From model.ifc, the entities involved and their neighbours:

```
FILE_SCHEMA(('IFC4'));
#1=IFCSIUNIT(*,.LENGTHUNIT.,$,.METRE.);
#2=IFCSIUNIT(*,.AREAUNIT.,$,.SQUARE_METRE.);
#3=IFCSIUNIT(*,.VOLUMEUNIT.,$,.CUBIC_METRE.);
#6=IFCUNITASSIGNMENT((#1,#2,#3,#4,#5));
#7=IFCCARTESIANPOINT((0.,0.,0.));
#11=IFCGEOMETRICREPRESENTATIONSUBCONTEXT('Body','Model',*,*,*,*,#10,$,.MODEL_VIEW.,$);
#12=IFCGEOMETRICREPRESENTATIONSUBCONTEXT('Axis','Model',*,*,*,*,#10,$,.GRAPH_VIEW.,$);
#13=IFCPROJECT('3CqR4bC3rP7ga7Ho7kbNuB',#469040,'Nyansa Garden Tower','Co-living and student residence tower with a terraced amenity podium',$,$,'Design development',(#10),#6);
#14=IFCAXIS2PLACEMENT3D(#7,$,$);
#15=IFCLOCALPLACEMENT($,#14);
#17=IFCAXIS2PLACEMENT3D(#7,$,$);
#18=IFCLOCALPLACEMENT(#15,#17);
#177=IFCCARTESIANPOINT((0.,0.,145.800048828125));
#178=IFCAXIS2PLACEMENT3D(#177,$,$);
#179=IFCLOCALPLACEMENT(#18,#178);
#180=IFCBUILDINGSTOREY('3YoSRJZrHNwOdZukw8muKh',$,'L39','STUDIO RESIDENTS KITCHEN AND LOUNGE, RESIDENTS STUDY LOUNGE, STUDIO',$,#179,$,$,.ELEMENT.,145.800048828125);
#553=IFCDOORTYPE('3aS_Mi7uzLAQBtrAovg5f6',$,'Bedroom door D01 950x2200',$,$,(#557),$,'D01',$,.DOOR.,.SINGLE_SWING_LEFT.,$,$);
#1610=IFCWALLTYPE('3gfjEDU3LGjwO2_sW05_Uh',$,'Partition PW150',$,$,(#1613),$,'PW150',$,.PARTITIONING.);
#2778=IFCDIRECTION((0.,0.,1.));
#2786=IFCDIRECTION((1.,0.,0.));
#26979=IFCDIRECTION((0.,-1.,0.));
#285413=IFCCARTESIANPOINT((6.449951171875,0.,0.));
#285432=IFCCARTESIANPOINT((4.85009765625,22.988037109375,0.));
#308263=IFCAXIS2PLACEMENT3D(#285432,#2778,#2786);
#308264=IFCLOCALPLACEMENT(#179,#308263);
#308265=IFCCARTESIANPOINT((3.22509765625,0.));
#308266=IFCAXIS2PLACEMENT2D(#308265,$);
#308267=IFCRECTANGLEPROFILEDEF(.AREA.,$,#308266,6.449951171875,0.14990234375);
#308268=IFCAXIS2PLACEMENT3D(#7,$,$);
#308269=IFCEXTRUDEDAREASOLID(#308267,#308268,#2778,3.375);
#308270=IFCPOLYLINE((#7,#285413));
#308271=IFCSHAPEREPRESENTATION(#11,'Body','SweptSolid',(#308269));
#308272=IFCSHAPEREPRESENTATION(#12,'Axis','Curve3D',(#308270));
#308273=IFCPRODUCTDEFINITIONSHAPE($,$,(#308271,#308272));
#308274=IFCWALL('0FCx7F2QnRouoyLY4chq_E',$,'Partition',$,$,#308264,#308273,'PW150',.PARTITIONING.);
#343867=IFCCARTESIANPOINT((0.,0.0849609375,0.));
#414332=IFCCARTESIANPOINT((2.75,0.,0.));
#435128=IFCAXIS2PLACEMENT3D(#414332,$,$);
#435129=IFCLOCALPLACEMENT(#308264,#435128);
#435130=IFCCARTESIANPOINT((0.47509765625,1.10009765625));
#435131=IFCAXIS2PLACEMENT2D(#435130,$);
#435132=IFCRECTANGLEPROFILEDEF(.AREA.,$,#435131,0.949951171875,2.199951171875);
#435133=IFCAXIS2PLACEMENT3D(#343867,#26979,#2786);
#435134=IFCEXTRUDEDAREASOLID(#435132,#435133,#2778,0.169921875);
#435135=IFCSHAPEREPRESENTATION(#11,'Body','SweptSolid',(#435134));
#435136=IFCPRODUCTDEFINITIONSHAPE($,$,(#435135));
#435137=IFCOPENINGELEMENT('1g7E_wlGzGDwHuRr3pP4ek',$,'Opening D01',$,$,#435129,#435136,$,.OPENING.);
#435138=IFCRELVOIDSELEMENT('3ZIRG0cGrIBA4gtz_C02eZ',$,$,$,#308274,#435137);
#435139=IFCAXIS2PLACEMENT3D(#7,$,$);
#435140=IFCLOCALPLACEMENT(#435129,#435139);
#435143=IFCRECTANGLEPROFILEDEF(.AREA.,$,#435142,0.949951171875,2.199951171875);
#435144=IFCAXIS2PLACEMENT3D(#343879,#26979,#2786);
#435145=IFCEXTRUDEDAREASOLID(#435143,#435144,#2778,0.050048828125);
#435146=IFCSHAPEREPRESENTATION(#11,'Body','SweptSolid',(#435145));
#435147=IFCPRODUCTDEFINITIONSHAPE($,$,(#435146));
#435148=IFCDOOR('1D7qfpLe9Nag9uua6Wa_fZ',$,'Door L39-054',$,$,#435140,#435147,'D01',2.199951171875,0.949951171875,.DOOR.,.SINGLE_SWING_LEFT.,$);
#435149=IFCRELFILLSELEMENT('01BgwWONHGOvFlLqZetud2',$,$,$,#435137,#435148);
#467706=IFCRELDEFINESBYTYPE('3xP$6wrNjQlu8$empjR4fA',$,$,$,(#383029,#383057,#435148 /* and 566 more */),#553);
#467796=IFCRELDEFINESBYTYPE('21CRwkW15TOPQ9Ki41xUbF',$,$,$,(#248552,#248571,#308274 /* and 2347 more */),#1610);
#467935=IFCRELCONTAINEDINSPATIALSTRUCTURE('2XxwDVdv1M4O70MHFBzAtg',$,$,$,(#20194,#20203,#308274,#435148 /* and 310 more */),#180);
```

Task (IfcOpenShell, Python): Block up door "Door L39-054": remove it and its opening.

```python
import ifcopenshell
import ifcopenshell.api.feature
import ifcopenshell.api.root
import ifcopenshell.geom
import ifcopenshell.util.shape

model = ifcopenshell.open("model.ifc")
settings = ifcopenshell.geom.settings()


def volume(element):
    """Net volume in cubic metres, openings subtracted."""
    shape = ifcopenshell.geom.create_shape(settings, element)
    return ifcopenshell.util.shape.get_volume(shape.geometry)


door = model.by_guid("1D7qfpLe9Nag9uua6Wa_fZ")
opening = door.FillsVoids[0].RelatingOpeningElement
wall = opening.VoidsElements[0].RelatingBuildingElement
before = volume(wall)

ifcopenshell.api.root.remove_product(model, product=door)
ifcopenshell.api.feature.remove_feature(model, feature=opening)

after = volume(wall)

print(f"wall volume {before:.3f} -> {after:.3f} m3")

model.write("model_edited.ifc")
```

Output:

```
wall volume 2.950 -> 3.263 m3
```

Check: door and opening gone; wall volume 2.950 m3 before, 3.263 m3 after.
